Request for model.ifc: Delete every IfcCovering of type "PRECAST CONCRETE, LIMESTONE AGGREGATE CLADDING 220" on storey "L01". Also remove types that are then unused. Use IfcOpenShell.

First a look at what the model holds.

```python
import ifcopenshell
import ifcopenshell.util.element

model = ifcopenshell.open("model.ifc")
print(model.schema)
storey = next(s for s in model.by_type("IfcBuildingStorey") if s.Name == "L01")
coverings = [e for e in ifcopenshell.util.element.get_decomposition(storey) if e.is_a("IfcCovering")]
seen = {}
for e in coverings:
    element_type = ifcopenshell.util.element.get_type(e)
    name = element_type.Name if element_type not in (None, e) else None
    seen[name] = seen.get(name, 0) + 1
for name, count in sorted(seen.items(), key=str):
    print(count, "x", name)
```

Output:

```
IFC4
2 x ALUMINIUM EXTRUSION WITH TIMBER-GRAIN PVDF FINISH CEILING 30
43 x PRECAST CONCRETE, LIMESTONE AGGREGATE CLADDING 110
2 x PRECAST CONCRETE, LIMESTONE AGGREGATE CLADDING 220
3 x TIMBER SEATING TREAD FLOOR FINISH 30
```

```python
import ifcopenshell
import ifcopenshell.api.root
import ifcopenshell.util.element

model = ifcopenshell.open("model.ifc")

storey = next(s for s in model.by_type("IfcBuildingStorey") if s.Name == "L01")
coverings = [e for e in ifcopenshell.util.element.get_decomposition(storey) if e.is_a("IfcCovering")]
targets = [e for e in coverings if (t := ifcopenshell.util.element.get_type(e)) not in (None, e) and t.Name == "PRECAST CONCRETE, LIMESTONE AGGREGATE CLADDING 220"]
types = {ifcopenshell.util.element.get_type(e) for e in targets} - {None, *targets}

for e in targets:
    ifcopenshell.api.root.remove_product(model, product=e)
print(len(targets), "removed")

unused = [t for t in types if not ifcopenshell.util.element.get_types(t)]
for t in unused:
    ifcopenshell.api.root.remove_product(model, product=t)
print(len(unused), "unused types removed")

model.write("model_edited.ifc")
```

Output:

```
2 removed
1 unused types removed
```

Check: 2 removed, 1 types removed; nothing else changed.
